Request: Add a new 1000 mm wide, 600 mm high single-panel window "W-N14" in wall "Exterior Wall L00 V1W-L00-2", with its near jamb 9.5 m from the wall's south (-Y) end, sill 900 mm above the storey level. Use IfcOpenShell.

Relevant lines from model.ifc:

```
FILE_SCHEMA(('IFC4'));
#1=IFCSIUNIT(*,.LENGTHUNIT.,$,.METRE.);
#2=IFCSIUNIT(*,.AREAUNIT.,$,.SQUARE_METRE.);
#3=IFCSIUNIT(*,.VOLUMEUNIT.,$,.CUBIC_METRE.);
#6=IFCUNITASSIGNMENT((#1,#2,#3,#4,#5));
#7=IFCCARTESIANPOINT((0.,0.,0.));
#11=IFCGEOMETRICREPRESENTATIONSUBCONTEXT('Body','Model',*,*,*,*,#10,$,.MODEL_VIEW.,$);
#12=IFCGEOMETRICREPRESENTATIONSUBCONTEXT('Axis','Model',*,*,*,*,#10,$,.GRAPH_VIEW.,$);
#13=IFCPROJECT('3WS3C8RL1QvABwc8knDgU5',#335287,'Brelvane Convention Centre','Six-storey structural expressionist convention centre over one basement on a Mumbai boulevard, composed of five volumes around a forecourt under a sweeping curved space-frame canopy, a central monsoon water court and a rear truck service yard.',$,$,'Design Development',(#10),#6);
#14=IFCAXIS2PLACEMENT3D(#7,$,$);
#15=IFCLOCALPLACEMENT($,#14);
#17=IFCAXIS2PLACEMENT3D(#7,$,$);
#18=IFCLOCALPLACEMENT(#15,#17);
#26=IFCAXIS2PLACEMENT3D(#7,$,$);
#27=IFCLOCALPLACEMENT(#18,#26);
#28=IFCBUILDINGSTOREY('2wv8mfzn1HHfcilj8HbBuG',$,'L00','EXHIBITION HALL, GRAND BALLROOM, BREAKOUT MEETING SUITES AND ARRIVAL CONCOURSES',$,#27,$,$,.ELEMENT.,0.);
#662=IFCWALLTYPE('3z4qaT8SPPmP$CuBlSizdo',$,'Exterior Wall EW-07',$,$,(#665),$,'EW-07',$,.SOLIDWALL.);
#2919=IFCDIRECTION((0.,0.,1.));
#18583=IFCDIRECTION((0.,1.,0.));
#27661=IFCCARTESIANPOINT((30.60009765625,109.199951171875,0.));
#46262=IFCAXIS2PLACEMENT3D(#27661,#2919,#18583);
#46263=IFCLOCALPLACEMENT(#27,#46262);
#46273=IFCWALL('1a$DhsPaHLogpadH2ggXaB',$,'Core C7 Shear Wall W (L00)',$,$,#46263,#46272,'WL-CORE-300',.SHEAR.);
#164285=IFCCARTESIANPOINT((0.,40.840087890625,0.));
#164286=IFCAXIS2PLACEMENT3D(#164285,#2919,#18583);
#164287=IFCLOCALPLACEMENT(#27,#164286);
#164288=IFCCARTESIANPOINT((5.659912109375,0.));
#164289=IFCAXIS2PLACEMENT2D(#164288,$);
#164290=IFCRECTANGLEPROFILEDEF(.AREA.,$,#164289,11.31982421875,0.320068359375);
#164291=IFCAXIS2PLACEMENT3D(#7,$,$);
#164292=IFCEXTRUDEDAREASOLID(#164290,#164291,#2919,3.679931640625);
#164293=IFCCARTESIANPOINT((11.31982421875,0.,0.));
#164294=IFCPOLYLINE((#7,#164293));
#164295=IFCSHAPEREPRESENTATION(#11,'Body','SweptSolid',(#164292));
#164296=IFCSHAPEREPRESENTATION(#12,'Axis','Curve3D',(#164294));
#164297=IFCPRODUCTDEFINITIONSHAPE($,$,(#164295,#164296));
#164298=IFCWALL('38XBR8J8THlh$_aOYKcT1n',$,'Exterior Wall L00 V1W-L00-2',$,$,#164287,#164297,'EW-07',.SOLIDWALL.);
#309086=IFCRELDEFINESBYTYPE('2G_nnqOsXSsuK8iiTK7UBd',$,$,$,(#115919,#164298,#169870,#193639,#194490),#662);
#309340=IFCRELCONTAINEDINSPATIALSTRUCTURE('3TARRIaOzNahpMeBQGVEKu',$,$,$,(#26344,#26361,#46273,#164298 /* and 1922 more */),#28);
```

```python
import numpy as np
import ifcopenshell
import ifcopenshell.api.feature
import ifcopenshell.api.geometry
import ifcopenshell.api.root
import ifcopenshell.api.spatial
import ifcopenshell.geom
import ifcopenshell.util.element
import ifcopenshell.util.placement
import ifcopenshell.util.representation
import ifcopenshell.util.shape
import ifcopenshell.util.unit

model = ifcopenshell.open("model.ifc")
unit_scale = ifcopenshell.util.unit.calculate_unit_scale(model)
settings = ifcopenshell.geom.settings()


def volume(element):
    """Net volume in cubic metres, openings subtracted."""
    shape = ifcopenshell.geom.create_shape(settings, element)
    return ifcopenshell.util.shape.get_volume(shape.geometry)


wall = model.by_guid("38XBR8J8THlh$_aOYKcT1n")
storey = ifcopenshell.util.element.get_container(wall, ifc_class="IfcBuildingStorey")
context = ifcopenshell.util.representation.get_context(model, "Model", "Body", "MODEL_VIEW")
before = volume(wall)

width, height, from_end, sill = 1, 0.6, 9.5, 0.9  # metres

# The wall runs along its own X axis, and the end named is its -X end.
wall_shape = ifcopenshell.geom.create_shape(settings, wall)
x, y, z = ifcopenshell.util.shape.get_vertices(wall_shape.geometry).T
start = x.min() + from_end
face, thickness = float(y.min()), float(y.max() - y.min())
wall_matrix = ifcopenshell.util.placement.get_local_placement(wall.ObjectPlacement)
level = ifcopenshell.util.placement.get_local_placement(storey.ObjectPlacement)[2, 3]


def in_wall(x, y):
    """Placement at x, y metres in the wall's axes, at sill height."""
    matrix = wall_matrix.copy()
    matrix[:, 3] = wall_matrix @ np.array([x / unit_scale, y / unit_scale, 0.0, 1.0])
    matrix[2, 3] = level + sill / unit_scale
    return matrix


# Opening: a box that overshoots both wall faces by 50 mm.
opening = ifcopenshell.api.root.create_entity(model, ifc_class="IfcOpeningElement", predefined_type="OPENING")
box = ifcopenshell.api.geometry.add_wall_representation(
    model, context=context, length=width, height=height, thickness=thickness + 0.1
)
ifcopenshell.api.geometry.assign_representation(model, product=opening, representation=box)
ifcopenshell.api.geometry.edit_object_placement(model, product=opening, matrix=in_wall(start, face - 0.05), is_si=False)
ifcopenshell.api.feature.add_feature(model, feature=opening, element=wall)

window = ifcopenshell.api.root.create_entity(model, ifc_class="IfcWindow", name="W-N14", predefined_type="WINDOW")
window.OverallWidth, window.OverallHeight = width / unit_scale, height / unit_scale
window.PartitioningType = "SINGLE_PANEL"
body = ifcopenshell.api.geometry.add_window_representation(
    model,
    context=context,
    overall_width=window.OverallWidth,
    overall_height=window.OverallHeight,
    partition_type="SINGLE_PANEL",
)
ifcopenshell.api.geometry.assign_representation(model, product=window, representation=body)
ifcopenshell.api.spatial.assign_container(model, products=[window], relating_structure=storey)
ifcopenshell.api.feature.add_filling(model, opening=opening, element=window)

# Centre the window in the wall's thickness.
ifcopenshell.api.geometry.edit_object_placement(model, product=window, matrix=in_wall(start, face), is_si=False)
window_shape = ifcopenshell.geom.create_shape(settings, window)
depth = ifcopenshell.util.shape.get_vertices(window_shape.geometry)[:, 1]
offset = face + thickness / 2 - (depth.min() + depth.max()) / 2
ifcopenshell.api.geometry.edit_object_placement(model, product=window, matrix=in_wall(start, offset), is_si=False)

after = volume(wall)

print(f"wall volume {before:.3f} -> {after:.3f} m3")

model.write("model-out.ifc")
```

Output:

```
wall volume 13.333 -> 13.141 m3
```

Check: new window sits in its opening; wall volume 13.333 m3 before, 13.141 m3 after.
